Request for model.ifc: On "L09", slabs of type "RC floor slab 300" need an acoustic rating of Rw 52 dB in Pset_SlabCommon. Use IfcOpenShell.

First a look at what the model holds.

```python
import ifcopenshell
import ifcopenshell.util.element

model = ifcopenshell.open("model.ifc")
print(model.schema)
storey = next(s for s in model.by_type("IfcBuildingStorey") if s.Name == "L09")
slabs = [e for e in ifcopenshell.util.element.get_decomposition(storey) if e.is_a("IfcSlab")]
seen = {}
for e in slabs:
    element_type = ifcopenshell.util.element.get_type(e)
    key = (element_type.Name if element_type != e and element_type else None, ifcopenshell.util.element.get_pset(e, "Pset_SlabCommon", "AcousticRating"))
    seen[key] = seen.get(key, 0) + 1
for (name, value), count in sorted(seen.items(), key=str):
    print(count, "x", name, "|", value)
```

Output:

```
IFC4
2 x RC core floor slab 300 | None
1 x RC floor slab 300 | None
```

```python
import ifcopenshell
import ifcopenshell.api.pset
import ifcopenshell.util.element

model = ifcopenshell.open("model.ifc")

storey = next(s for s in model.by_type("IfcBuildingStorey") if s.Name == "L09")
slabs = [e for e in ifcopenshell.util.element.get_decomposition(storey) if e.is_a("IfcSlab")]

count = 0
for e in slabs:
    element_type = ifcopenshell.util.element.get_type(e)
    if element_type in (None, e) or element_type.Name != "RC floor slab 300":
        continue
    # add_pset returns the element's existing set when there is one.
    pset = ifcopenshell.api.pset.add_pset(model, product=e, name="Pset_SlabCommon")
    ifcopenshell.api.pset.edit_pset(model, pset=pset, properties={"AcousticRating": "Rw 52 dB"})
    count += 1

print(count, "slabs updated")

model.write("model_rev.ifc")
```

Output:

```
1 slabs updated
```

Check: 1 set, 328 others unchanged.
